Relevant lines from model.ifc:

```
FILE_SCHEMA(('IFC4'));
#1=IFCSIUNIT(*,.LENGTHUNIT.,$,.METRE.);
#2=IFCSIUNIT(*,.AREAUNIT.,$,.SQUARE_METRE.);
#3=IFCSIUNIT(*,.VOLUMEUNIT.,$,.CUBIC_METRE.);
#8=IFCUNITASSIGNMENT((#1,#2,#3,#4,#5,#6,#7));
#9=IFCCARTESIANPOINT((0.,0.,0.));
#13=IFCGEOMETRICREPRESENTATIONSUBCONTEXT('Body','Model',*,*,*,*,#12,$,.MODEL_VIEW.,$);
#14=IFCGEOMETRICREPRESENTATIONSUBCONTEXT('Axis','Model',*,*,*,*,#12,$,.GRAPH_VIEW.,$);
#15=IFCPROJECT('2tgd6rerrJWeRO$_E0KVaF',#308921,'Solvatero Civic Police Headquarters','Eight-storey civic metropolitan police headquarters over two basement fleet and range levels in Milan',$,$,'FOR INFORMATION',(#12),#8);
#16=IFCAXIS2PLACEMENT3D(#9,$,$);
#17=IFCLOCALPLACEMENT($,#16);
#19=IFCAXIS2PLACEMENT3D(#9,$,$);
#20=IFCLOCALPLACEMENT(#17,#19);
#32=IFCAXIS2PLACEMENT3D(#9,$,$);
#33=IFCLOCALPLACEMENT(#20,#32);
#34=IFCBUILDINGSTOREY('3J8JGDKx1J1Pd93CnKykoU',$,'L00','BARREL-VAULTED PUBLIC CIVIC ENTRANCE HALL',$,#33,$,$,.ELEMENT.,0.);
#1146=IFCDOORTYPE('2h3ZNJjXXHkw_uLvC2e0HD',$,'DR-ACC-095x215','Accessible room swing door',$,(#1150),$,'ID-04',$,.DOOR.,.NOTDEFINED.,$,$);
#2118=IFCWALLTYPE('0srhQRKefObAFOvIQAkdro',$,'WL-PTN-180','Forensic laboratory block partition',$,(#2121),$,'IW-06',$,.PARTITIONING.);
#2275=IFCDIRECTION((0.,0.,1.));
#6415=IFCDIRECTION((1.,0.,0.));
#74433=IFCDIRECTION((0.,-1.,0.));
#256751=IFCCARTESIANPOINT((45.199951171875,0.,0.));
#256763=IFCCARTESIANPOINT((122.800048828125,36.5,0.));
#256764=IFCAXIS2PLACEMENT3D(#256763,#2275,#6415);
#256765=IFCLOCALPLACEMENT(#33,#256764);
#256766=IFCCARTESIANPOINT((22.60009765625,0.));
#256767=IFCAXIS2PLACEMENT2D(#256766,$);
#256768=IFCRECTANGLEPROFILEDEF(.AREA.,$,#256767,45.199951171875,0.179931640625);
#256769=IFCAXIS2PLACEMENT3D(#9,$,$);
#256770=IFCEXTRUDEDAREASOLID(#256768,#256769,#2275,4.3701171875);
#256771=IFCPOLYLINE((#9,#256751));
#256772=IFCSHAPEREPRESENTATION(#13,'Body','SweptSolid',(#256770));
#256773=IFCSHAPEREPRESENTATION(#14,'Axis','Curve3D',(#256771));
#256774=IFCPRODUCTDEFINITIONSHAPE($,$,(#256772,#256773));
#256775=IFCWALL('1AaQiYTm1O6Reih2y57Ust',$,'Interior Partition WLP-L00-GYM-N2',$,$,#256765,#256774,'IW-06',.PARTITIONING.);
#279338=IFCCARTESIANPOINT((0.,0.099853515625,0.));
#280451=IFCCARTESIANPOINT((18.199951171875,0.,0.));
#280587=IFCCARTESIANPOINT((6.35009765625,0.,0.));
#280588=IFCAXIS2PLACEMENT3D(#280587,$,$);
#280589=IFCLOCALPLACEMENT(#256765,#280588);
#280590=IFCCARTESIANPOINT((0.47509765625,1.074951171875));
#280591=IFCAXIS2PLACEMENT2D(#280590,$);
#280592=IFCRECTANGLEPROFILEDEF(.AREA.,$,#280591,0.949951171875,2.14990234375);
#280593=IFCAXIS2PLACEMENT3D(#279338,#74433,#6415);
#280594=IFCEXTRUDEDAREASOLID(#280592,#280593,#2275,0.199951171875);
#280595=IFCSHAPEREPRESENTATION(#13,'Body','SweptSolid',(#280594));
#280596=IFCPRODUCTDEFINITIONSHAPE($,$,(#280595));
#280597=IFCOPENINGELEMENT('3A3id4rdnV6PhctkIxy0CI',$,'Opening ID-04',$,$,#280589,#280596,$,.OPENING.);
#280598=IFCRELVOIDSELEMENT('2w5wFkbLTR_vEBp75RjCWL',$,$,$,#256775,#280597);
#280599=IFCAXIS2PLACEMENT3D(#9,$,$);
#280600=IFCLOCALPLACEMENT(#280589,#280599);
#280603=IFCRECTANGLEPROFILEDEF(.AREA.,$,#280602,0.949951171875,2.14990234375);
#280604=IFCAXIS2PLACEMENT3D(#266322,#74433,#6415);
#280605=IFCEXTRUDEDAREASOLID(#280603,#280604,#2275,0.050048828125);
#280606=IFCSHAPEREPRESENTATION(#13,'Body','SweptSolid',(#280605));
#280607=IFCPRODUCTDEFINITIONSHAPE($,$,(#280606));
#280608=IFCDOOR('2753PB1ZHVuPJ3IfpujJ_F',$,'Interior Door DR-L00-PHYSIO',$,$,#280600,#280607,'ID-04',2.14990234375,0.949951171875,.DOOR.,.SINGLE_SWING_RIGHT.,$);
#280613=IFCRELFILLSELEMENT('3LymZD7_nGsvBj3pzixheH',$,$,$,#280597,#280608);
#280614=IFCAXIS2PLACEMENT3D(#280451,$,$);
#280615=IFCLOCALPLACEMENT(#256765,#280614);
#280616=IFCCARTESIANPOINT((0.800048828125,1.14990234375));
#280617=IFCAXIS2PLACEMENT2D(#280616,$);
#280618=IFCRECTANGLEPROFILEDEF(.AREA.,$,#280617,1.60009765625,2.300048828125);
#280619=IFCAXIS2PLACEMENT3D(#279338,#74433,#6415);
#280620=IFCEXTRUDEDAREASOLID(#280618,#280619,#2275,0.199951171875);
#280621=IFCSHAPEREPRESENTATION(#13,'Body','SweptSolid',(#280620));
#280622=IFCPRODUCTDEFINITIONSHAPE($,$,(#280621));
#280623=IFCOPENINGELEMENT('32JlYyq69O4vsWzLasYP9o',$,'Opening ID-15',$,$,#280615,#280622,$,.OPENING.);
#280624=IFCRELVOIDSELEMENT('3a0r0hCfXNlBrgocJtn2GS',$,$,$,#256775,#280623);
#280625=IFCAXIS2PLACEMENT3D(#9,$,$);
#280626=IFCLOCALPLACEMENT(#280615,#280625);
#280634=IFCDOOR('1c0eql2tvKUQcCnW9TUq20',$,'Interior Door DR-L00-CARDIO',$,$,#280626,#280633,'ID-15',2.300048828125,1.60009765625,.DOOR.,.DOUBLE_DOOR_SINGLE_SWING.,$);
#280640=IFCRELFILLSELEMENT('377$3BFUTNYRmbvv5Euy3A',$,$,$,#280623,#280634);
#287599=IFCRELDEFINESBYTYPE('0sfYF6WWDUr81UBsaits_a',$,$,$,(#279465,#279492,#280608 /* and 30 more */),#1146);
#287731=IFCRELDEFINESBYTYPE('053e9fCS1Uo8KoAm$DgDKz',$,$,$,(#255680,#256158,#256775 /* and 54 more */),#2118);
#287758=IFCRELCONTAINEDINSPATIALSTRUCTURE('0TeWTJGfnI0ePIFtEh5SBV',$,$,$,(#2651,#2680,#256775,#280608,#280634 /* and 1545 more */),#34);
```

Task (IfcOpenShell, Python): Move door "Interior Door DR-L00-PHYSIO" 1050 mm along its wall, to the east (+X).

```python
import ifcopenshell
import ifcopenshell.api.geometry
import ifcopenshell.util.placement

model = ifcopenshell.open("model.ifc")

door = model.by_id(280608)
opening = door.FillsVoids[0].RelatingOpeningElement
wall = opening.VoidsElements[0].RelatingBuildingElement

wall_matrix = ifcopenshell.util.placement.get_local_placement(wall.ObjectPlacement)
shift = wall_matrix[:3, 0] * 1.05
before = ifcopenshell.util.placement.get_local_placement(door.ObjectPlacement)[:3, 3].copy()

# The door is placed relative to its opening, so it follows when the opening moves.
matrix = ifcopenshell.util.placement.get_local_placement(opening.ObjectPlacement)
matrix[:3, 3] += shift
ifcopenshell.api.geometry.edit_object_placement(
    model, product=opening, matrix=matrix, is_si=False, should_transform_children=True
)

after = ifcopenshell.util.placement.get_local_placement(door.ObjectPlacement)[:3, 3]
print("door moved by", (after - before).round(3) + 0.0)

model.write("model_edited.ifc")
```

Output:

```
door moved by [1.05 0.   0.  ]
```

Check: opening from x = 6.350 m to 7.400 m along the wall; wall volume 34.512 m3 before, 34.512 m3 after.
